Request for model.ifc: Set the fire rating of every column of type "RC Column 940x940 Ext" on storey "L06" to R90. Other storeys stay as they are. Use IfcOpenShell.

First a look at what the model holds.

```python
import ifcopenshell
import ifcopenshell.util.element

model = ifcopenshell.open("model.ifc")
print(model.schema)
storey = next(s for s in model.by_type("IfcBuildingStorey") if s.Name == "L06")
columns = [e for e in ifcopenshell.util.element.get_decomposition(storey) if e.is_a("IfcColumn")]
seen = {}
for e in columns:
    element_type = ifcopenshell.util.element.get_type(e)
    key = (element_type.Name if element_type != e and element_type else None, ifcopenshell.util.element.get_pset(e, "Pset_ColumnCommon", "FireRating"))
    seen[key] = seen.get(key, 0) + 1
for (name, value), count in sorted(seen.items(), key=str):
    print(count, "x", name, "|", value)
```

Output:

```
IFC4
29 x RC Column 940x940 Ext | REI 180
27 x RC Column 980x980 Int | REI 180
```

```python
import ifcopenshell
import ifcopenshell.api.pset
import ifcopenshell.util.element

model = ifcopenshell.open("model.ifc")

storey = next(s for s in model.by_type("IfcBuildingStorey") if s.Name == "L06")
columns = [e for e in ifcopenshell.util.element.get_decomposition(storey) if e.is_a("IfcColumn")]

count = 0
for e in columns:
    element_type = ifcopenshell.util.element.get_type(e)
    if element_type in (None, e) or element_type.Name != "RC Column 940x940 Ext":
        continue
    # add_pset returns the element's existing set when there is one.
    pset = ifcopenshell.api.pset.add_pset(model, product=e, name="Pset_ColumnCommon")
    ifcopenshell.api.pset.edit_pset(model, pset=pset, properties={"FireRating": "R90"})
    count += 1

print(count, "columns updated")

model.write("model_v2.ifc")
```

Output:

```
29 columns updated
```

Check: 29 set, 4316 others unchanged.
